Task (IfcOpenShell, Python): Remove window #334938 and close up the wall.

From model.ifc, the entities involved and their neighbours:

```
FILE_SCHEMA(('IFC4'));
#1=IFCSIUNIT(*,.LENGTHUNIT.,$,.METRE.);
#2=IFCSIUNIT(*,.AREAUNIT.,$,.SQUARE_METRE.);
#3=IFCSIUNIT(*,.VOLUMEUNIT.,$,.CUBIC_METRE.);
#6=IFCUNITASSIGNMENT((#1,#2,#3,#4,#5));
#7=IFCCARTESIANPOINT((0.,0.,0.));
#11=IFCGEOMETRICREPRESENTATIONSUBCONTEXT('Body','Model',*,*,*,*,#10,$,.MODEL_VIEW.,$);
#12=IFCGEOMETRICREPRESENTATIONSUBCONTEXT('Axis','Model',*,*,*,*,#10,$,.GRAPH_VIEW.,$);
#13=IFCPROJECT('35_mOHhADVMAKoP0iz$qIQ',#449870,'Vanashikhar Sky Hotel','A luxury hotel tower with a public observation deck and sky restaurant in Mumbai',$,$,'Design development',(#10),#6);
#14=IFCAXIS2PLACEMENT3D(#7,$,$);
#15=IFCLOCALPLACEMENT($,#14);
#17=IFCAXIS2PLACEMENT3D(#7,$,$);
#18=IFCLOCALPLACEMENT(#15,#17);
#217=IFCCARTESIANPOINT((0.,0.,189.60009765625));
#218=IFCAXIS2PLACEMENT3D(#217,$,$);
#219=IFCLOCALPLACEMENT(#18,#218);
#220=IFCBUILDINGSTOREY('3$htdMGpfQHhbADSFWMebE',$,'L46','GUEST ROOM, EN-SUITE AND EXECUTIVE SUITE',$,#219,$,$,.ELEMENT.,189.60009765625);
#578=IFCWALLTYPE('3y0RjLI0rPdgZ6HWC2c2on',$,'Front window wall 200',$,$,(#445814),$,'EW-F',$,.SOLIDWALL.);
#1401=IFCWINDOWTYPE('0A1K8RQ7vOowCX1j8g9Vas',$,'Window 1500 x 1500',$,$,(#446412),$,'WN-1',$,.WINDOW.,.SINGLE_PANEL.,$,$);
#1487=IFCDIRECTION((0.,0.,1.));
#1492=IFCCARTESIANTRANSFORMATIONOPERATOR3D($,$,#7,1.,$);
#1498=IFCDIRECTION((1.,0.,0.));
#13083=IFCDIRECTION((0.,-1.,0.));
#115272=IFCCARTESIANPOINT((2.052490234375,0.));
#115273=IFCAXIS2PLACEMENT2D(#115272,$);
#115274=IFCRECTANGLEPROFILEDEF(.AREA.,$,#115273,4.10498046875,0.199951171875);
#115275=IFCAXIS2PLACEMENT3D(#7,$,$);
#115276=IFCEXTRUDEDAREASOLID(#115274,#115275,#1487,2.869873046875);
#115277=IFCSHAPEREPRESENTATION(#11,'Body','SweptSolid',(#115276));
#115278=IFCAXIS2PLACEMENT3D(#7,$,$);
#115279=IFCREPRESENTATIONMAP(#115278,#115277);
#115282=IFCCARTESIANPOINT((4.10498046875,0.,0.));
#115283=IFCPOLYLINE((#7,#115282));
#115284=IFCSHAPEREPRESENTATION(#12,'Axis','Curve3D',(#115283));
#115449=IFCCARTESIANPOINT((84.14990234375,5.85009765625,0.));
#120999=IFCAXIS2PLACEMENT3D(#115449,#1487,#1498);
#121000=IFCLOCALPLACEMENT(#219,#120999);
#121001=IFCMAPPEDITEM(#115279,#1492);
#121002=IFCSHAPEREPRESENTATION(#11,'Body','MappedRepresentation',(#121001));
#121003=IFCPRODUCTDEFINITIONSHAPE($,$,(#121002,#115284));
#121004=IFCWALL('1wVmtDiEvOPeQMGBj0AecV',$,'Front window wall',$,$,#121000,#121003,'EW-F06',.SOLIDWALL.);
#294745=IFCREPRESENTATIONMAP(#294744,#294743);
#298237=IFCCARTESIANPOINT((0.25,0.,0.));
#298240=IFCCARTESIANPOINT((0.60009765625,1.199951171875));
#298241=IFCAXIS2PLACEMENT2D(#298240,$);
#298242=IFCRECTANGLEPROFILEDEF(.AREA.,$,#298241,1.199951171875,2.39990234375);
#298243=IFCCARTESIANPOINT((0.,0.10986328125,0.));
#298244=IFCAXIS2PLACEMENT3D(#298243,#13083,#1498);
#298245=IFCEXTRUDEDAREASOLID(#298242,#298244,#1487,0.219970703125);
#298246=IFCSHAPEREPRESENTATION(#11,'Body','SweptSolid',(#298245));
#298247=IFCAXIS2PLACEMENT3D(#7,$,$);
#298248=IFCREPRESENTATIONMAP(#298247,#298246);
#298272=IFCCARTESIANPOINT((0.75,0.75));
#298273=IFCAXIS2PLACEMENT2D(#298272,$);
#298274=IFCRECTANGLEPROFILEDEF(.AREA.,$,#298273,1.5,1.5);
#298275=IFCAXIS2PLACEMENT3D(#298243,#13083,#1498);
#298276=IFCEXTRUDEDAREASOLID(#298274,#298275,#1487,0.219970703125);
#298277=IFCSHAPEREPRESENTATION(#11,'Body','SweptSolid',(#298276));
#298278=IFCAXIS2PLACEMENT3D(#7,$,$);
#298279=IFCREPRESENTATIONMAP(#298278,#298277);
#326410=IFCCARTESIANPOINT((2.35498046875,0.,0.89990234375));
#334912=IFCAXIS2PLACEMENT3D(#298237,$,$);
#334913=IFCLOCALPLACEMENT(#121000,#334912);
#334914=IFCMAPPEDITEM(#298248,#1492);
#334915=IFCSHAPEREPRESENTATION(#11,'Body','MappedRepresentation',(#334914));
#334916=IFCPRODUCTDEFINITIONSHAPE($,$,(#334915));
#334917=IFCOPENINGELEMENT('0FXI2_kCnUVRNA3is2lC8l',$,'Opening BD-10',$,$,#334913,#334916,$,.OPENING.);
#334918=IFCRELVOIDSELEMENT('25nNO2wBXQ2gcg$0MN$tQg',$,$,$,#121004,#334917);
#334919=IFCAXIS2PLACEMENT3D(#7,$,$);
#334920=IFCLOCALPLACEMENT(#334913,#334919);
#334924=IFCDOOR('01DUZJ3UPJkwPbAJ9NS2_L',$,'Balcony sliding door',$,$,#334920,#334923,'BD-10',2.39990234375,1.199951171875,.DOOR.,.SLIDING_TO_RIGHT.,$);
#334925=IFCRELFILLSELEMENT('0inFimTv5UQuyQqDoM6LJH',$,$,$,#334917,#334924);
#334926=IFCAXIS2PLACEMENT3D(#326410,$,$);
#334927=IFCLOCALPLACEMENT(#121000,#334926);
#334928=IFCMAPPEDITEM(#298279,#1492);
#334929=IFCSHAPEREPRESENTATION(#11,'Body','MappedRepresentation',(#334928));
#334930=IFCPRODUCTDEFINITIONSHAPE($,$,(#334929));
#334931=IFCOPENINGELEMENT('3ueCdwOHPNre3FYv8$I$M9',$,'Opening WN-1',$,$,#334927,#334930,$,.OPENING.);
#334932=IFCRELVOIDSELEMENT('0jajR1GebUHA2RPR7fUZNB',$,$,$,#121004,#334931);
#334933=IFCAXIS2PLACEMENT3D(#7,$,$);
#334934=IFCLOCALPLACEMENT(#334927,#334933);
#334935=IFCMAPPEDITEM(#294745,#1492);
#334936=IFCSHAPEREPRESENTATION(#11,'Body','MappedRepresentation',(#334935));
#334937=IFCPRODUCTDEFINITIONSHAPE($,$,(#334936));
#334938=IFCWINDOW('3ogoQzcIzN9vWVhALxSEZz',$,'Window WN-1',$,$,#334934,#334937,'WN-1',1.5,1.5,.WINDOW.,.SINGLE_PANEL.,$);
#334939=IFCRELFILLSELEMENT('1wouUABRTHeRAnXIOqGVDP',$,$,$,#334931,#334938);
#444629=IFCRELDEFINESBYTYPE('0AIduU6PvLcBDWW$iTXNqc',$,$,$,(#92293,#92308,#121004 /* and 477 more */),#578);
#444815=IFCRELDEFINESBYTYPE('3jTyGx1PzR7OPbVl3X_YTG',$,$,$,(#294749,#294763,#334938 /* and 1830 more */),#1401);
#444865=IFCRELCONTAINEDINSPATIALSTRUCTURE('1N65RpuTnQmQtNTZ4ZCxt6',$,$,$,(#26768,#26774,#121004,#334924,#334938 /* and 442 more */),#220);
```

```python
import ifcopenshell
import ifcopenshell.api.feature
import ifcopenshell.api.root
import ifcopenshell.geom
import ifcopenshell.util.shape

model = ifcopenshell.open("model.ifc")
settings = ifcopenshell.geom.settings()


def volume(element):
    """Net volume in cubic metres, openings subtracted."""
    shape = ifcopenshell.geom.create_shape(settings, element)
    return ifcopenshell.util.shape.get_volume(shape.geometry)


window = model.by_guid("3ogoQzcIzN9vWVhALxSEZz")
opening = window.FillsVoids[0].RelatingOpeningElement
wall = opening.VoidsElements[0].RelatingBuildingElement
before = volume(wall)

ifcopenshell.api.root.remove_product(model, product=window)
ifcopenshell.api.feature.remove_feature(model, feature=opening)

after = volume(wall)

print(f"wall volume {before:.3f} -> {after:.3f} m3")

model.write("model_v2.ifc")
```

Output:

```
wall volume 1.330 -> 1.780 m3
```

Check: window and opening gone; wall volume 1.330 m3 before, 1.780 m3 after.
